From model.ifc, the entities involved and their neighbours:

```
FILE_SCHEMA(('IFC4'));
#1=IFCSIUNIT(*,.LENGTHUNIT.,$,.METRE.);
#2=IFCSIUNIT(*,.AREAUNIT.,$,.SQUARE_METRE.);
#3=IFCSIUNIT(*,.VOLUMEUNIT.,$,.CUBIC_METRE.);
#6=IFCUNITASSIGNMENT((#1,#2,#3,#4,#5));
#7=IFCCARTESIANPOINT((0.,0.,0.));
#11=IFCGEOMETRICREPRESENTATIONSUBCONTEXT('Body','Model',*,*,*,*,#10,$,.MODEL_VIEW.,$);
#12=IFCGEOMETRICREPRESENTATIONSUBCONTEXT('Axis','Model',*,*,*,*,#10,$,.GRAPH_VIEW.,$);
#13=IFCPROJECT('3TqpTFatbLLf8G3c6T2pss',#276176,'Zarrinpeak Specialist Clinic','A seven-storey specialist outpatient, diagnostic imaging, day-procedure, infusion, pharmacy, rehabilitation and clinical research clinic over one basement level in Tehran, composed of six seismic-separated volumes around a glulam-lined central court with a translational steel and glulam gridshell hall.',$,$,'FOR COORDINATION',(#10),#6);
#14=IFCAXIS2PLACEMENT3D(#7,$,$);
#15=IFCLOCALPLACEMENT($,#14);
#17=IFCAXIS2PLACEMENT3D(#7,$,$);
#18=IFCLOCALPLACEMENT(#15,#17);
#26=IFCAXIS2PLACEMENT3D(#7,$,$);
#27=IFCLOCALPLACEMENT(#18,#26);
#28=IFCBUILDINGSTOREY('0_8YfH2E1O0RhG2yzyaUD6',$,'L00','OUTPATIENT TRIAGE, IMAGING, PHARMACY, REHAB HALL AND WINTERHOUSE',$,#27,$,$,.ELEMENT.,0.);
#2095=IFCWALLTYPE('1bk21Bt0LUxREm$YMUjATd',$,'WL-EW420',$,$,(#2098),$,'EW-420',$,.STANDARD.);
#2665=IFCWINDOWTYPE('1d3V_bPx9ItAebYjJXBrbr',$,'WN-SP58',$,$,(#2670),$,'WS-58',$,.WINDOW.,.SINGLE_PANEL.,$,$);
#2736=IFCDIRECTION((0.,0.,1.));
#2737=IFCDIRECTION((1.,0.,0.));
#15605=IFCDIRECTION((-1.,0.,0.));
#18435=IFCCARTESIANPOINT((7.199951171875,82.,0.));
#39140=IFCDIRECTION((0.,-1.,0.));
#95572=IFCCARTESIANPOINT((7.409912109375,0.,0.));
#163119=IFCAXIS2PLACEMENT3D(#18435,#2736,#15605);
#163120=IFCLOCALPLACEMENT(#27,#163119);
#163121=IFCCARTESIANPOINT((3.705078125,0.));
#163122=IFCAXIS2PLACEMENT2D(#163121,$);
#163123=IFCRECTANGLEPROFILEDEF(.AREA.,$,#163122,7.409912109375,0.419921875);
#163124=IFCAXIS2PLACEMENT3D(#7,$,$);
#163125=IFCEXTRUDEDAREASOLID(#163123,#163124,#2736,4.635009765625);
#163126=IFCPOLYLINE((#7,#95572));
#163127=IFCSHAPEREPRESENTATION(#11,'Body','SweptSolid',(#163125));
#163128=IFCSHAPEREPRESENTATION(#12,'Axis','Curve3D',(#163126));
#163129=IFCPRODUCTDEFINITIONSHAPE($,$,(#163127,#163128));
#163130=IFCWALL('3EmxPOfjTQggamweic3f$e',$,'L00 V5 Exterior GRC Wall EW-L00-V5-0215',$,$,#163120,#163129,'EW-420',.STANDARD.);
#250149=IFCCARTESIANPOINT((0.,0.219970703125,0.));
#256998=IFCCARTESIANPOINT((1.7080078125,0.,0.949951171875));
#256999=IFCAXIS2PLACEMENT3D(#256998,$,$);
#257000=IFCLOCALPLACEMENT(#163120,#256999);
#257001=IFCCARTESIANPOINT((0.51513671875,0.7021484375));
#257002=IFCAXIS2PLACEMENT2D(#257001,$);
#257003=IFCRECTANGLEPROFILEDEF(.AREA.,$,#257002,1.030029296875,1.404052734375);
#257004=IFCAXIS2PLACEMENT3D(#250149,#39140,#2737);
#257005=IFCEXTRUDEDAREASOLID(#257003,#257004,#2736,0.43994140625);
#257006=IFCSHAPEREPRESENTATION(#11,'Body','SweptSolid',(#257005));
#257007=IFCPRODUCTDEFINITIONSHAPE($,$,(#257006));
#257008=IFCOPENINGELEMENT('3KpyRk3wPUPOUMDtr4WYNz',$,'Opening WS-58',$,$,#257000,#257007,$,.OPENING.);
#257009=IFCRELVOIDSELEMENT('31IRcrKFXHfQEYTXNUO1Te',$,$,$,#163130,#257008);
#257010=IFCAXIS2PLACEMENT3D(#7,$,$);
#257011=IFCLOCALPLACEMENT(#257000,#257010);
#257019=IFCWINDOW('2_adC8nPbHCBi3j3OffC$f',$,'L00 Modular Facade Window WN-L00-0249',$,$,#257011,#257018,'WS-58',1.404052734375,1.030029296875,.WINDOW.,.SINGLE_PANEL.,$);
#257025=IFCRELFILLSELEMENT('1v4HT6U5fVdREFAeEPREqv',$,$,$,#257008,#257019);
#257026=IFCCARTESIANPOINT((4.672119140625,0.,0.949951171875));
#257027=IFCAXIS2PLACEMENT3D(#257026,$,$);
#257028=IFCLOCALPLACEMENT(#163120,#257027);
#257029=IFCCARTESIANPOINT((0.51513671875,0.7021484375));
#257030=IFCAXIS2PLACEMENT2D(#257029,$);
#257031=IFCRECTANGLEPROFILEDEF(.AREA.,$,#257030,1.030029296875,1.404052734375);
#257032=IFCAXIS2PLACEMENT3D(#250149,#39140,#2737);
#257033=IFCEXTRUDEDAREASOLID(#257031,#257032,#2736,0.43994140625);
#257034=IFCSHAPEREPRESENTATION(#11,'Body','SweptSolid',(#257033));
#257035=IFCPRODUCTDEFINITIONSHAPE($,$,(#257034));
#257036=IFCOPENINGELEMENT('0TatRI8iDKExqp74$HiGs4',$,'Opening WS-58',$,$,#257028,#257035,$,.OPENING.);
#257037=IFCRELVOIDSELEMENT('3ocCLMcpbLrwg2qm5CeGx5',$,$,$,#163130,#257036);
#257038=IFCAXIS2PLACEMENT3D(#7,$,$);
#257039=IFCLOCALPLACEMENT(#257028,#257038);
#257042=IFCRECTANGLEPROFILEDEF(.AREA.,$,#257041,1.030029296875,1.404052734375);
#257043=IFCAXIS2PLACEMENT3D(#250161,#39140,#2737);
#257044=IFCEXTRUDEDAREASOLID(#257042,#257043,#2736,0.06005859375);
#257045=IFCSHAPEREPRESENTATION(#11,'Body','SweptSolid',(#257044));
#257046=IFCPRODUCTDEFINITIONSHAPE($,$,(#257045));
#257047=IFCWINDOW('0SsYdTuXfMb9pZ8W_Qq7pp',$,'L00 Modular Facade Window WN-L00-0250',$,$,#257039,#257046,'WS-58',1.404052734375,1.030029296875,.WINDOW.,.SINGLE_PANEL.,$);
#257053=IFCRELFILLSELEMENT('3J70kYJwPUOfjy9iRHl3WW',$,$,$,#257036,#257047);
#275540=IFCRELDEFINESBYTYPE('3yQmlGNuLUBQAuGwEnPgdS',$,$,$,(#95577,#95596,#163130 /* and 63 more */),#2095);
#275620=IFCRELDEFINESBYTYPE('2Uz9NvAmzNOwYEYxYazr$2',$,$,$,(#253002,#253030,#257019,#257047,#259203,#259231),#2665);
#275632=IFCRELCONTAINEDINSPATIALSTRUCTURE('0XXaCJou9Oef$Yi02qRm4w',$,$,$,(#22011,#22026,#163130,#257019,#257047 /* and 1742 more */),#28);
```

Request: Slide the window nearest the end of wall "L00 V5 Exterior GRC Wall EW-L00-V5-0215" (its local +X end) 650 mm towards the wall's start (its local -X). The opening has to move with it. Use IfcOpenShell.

```python
import ifcopenshell
import ifcopenshell.api.geometry
import ifcopenshell.util.placement
import ifcopenshell.util.unit

model = ifcopenshell.open("model.ifc")
unit_scale = ifcopenshell.util.unit.calculate_unit_scale(model)

window = model.by_guid("0SsYdTuXfMb9pZ8W_Qq7pp")
opening = window.FillsVoids[0].RelatingOpeningElement
wall = opening.VoidsElements[0].RelatingBuildingElement

wall_matrix = ifcopenshell.util.placement.get_local_placement(wall.ObjectPlacement)
shift = wall_matrix[:3, 0] * -0.65 / unit_scale
before = ifcopenshell.util.placement.get_local_placement(window.ObjectPlacement)[:3, 3].copy()

# The window is placed relative to its opening, so it follows when the opening moves.
matrix = ifcopenshell.util.placement.get_local_placement(opening.ObjectPlacement)
matrix[:3, 3] += shift
ifcopenshell.api.geometry.edit_object_placement(
    model, product=opening, matrix=matrix, is_si=False, should_transform_children=True
)

after = ifcopenshell.util.placement.get_local_placement(window.ObjectPlacement)[:3, 3]
print("window moved by", (after - before).round(3) + 0.0)

model.write("model-out.ifc")
```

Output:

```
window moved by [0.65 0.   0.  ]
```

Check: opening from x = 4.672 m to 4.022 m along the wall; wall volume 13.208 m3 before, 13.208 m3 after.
